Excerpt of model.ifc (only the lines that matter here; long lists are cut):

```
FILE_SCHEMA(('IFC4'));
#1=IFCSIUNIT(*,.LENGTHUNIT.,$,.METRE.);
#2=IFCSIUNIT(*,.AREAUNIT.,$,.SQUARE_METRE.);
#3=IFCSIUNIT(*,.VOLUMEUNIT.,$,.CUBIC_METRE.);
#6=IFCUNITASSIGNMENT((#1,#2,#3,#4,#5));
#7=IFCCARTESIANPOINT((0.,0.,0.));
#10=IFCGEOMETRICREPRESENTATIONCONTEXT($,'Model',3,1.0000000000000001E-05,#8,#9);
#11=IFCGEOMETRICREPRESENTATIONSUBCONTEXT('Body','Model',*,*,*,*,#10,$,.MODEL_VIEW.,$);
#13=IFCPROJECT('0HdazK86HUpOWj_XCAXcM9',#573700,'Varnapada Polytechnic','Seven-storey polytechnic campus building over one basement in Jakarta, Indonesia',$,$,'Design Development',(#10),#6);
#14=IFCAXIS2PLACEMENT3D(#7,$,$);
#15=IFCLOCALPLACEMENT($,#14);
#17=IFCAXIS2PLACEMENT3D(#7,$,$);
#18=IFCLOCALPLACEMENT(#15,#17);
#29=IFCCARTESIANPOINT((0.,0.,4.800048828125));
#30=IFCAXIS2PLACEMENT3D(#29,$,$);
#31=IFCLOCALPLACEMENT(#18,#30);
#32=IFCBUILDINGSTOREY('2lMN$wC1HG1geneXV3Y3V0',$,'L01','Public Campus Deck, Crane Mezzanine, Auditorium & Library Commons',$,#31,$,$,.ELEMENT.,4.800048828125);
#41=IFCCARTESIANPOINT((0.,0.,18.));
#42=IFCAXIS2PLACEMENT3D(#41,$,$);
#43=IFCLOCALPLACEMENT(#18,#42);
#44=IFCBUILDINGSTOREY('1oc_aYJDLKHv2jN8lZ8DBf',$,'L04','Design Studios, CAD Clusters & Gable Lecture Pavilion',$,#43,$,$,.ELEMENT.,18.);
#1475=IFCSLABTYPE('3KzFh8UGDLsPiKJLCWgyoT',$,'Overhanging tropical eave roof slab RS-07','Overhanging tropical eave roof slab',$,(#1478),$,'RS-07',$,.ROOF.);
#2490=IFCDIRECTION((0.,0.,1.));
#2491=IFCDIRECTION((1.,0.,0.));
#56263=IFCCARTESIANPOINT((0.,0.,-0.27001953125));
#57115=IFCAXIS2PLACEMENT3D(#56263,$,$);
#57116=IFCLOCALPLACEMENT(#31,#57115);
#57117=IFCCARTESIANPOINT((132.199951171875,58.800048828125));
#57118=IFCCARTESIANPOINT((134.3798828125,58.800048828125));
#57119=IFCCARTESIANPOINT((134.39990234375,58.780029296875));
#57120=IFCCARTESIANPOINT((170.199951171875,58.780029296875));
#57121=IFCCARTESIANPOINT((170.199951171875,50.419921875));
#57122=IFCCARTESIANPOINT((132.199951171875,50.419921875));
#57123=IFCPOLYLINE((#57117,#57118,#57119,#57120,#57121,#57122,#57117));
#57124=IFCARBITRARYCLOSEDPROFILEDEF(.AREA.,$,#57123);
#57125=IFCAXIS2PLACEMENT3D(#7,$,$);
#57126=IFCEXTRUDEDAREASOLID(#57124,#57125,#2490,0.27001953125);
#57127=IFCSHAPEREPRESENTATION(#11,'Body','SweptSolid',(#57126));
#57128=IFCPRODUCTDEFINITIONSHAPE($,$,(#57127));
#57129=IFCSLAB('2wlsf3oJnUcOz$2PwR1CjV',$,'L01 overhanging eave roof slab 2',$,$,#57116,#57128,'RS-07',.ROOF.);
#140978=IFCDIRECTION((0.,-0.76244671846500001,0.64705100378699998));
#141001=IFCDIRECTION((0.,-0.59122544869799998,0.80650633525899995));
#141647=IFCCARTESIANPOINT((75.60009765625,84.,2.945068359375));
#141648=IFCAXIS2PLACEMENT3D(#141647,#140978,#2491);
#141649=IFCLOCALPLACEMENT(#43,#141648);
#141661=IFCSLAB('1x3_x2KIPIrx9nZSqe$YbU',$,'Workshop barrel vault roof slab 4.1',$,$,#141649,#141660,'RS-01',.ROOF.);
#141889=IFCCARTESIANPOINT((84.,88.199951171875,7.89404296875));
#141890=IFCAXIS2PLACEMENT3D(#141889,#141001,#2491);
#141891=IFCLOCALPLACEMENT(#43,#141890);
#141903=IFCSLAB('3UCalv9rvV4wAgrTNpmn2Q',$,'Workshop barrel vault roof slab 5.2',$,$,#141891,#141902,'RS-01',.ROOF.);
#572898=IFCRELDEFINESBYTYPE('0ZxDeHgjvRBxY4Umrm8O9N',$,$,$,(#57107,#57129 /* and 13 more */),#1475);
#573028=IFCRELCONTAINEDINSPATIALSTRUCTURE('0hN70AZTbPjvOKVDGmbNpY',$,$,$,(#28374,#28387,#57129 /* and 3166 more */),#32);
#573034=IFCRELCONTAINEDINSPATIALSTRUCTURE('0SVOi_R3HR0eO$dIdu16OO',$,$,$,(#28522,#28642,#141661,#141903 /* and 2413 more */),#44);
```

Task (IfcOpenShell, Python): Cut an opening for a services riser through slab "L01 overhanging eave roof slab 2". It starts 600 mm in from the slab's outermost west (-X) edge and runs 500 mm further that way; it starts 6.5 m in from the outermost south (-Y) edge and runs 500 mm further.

```python
import numpy as np
import ifcopenshell
import ifcopenshell.api.feature
import ifcopenshell.api.geometry
import ifcopenshell.api.root
import ifcopenshell.geom
import ifcopenshell.util.placement
import ifcopenshell.util.representation
import ifcopenshell.util.shape
import ifcopenshell.util.unit

model = ifcopenshell.open("model.ifc")
unit_scale = ifcopenshell.util.unit.calculate_unit_scale(model)
settings = ifcopenshell.geom.settings()


def volume(element):
    """Net volume in cubic metres, openings subtracted."""
    shape = ifcopenshell.geom.create_shape(settings, element)
    return ifcopenshell.util.shape.get_volume(shape.geometry)


slab = model.by_id(57129)
before = volume(slab)

# Extent in the slab's own axes, in metres. The edges named are its -X and -Y sides.
slab_shape = ifcopenshell.geom.create_shape(settings, slab)
vertices = ifcopenshell.util.shape.get_vertices(slab_shape.geometry)
x_min, y_min, bottom = vertices.min(axis=0)
top = vertices[:, 2].max()

opening = ifcopenshell.api.root.create_entity(model, ifc_class="IfcOpeningElement", name="Services riser opening", predefined_type="OPENING")
context = ifcopenshell.util.representation.get_context(model, "Model", "Body", "MODEL_VIEW")
width, depth = 0.5, 0.5
outline = [(0.0, 0.0), (width, 0.0), (width, depth), (0.0, depth), (0.0, 0.0)]
# Overshoot both faces by 50 mm so the cut is clean.
shape = ifcopenshell.api.geometry.add_slab_representation(
    model, context=context, depth=top - bottom + 0.1, polyline=outline
)
ifcopenshell.api.geometry.assign_representation(model, product=opening, representation=shape)

matrix = ifcopenshell.util.placement.get_local_placement(slab.ObjectPlacement)
matrix[:, 3] = matrix @ np.append(np.array([x_min + 0.6, y_min + 6.5, bottom - 0.05]) / unit_scale, 1.0)
ifcopenshell.api.geometry.edit_object_placement(model, product=opening, matrix=matrix, is_si=False)
ifcopenshell.api.feature.add_feature(model, feature=opening, element=slab)

after = volume(slab)

print(f"slab volume {before:.3f} -> {after:.3f} m3")

model.write("model_updated.ifc")
```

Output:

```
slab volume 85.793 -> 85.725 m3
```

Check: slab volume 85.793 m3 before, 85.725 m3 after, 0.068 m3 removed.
